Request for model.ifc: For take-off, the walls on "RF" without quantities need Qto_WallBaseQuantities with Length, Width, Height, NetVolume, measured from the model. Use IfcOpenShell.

First a look at what the model holds.

```python
import ifcopenshell
import ifcopenshell.util.element
import ifcopenshell.util.unit

model = ifcopenshell.open("model.ifc")
print(model.schema)
for unit_type in ("LENGTHUNIT", "AREAUNIT", "VOLUMEUNIT"):
    print(unit_type, ifcopenshell.util.unit.calculate_unit_scale(model, unit_type))
storey = next(s for s in model.by_type("IfcBuildingStorey") if s.Name == "RF")
walls = [e for e in ifcopenshell.util.element.get_decomposition(storey) if e.is_a("IfcWall")]
for e in sorted(walls, key=lambda e: e.id()):
    print(e.id(), e.is_a(), e.Name, list(ifcopenshell.util.element.get_psets(e, qtos_only=True)), sep=" | ")
```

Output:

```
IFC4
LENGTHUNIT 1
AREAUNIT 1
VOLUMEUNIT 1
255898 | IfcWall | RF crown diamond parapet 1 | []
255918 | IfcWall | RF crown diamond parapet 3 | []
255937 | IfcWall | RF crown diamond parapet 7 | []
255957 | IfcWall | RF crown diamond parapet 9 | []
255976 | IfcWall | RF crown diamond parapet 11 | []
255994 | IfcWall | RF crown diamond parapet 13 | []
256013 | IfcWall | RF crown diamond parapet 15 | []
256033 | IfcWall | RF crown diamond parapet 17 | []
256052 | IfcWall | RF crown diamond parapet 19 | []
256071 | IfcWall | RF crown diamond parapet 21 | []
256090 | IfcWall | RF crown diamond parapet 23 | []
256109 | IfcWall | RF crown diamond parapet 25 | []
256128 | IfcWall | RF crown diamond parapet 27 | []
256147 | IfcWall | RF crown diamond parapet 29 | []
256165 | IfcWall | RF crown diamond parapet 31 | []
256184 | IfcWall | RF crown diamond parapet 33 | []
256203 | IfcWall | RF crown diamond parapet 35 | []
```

```python
import ifcopenshell
import ifcopenshell.api.pset
import ifcopenshell.geom
import ifcopenshell.util.element
import ifcopenshell.util.shape
import ifcopenshell.util.unit

model = ifcopenshell.open("model.ifc")
unit_scale = ifcopenshell.util.unit.calculate_unit_scale(model)
volume_scale = ifcopenshell.util.unit.calculate_unit_scale(model, "VOLUMEUNIT")
settings = ifcopenshell.geom.settings()

storey = next(s for s in model.by_type("IfcBuildingStorey") if s.Name == "RF")
walls = [e for e in ifcopenshell.util.element.get_decomposition(storey) if e.is_a("IfcWall")]

for e in sorted(walls, key=lambda e: e.id()):
    if ifcopenshell.util.element.get_psets(e, qtos_only=True, should_inherit=False):
        continue
    # Geometry comes back in metres, in the element's own axes.
    shape = ifcopenshell.geom.create_shape(settings, e)
    values = {
        "Length": ifcopenshell.util.shape.get_x(shape.geometry) / unit_scale,
        "Width": ifcopenshell.util.shape.get_y(shape.geometry) / unit_scale,
        "Height": ifcopenshell.util.shape.get_z(shape.geometry) / unit_scale,
        "NetVolume": ifcopenshell.util.shape.get_volume(shape.geometry) / volume_scale,
    }
    qto = ifcopenshell.api.pset.add_qto(model, product=e, name="Qto_WallBaseQuantities")
    ifcopenshell.api.pset.edit_qto(model, qto=qto, properties=values)
    print(e.id(), {k: round(v, 3) for k, v in values.items()})

model.write("model_updated.ifc")
```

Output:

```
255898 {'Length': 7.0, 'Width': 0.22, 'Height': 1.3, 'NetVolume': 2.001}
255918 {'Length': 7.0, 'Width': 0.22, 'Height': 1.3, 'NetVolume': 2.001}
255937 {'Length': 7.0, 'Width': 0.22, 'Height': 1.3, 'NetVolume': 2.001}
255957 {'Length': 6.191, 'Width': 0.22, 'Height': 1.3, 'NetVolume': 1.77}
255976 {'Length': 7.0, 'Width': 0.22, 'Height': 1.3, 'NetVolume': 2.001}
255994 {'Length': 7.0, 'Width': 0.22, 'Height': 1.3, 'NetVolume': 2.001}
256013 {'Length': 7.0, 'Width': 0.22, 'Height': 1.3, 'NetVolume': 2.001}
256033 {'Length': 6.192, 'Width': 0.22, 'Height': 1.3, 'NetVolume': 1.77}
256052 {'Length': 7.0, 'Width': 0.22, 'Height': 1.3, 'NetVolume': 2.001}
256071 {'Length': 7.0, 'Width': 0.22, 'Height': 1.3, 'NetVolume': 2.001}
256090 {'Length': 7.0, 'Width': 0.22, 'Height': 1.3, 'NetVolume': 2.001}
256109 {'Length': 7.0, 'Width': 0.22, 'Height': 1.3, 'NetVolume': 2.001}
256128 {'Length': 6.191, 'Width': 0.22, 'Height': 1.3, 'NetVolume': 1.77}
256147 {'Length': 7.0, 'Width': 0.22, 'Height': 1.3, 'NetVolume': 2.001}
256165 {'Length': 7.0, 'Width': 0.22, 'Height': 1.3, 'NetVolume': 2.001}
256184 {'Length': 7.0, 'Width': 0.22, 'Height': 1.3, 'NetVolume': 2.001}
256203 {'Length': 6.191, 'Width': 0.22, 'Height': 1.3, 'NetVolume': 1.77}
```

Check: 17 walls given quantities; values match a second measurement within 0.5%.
